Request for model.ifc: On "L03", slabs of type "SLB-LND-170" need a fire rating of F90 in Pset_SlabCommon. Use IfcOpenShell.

First a look at what the model holds.

```python
import ifcopenshell
import ifcopenshell.util.element

model = ifcopenshell.open("model.ifc")
print(model.schema)
storey = next(s for s in model.by_type("IfcBuildingStorey") if s.Name == "L03")
slabs = [e for e in ifcopenshell.util.element.get_decomposition(storey) if e.is_a("IfcSlab")]
seen = {}
for e in slabs:
    element_type = ifcopenshell.util.element.get_type(e)
    key = (element_type.Name if element_type != e and element_type else None, ifcopenshell.util.element.get_pset(e, "Pset_SlabCommon", "FireRating"))
    seen[key] = seen.get(key, 0) + 1
for (name, value), count in sorted(seen.items(), key=str):
    print(count, "x", name, "|", value)
```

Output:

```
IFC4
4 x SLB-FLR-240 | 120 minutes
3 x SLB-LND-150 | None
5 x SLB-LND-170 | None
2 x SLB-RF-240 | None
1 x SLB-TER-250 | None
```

```python
import ifcopenshell
import ifcopenshell.api.pset
import ifcopenshell.util.element

model = ifcopenshell.open("model.ifc")

storey = next(s for s in model.by_type("IfcBuildingStorey") if s.Name == "L03")
slabs = [e for e in ifcopenshell.util.element.get_decomposition(storey) if e.is_a("IfcSlab")]

count = 0
for e in slabs:
    element_type = ifcopenshell.util.element.get_type(e)
    if element_type in (None, e) or element_type.Name != "SLB-LND-170":
        continue
    # add_pset returns the element's existing set when there is one.
    pset = ifcopenshell.api.pset.add_pset(model, product=e, name="Pset_SlabCommon")
    ifcopenshell.api.pset.edit_pset(model, pset=pset, properties={"FireRating": "F90"})
    count += 1

print(count, "slabs updated")

model.write("model_edited.ifc")
```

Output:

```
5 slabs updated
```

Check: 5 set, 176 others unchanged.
